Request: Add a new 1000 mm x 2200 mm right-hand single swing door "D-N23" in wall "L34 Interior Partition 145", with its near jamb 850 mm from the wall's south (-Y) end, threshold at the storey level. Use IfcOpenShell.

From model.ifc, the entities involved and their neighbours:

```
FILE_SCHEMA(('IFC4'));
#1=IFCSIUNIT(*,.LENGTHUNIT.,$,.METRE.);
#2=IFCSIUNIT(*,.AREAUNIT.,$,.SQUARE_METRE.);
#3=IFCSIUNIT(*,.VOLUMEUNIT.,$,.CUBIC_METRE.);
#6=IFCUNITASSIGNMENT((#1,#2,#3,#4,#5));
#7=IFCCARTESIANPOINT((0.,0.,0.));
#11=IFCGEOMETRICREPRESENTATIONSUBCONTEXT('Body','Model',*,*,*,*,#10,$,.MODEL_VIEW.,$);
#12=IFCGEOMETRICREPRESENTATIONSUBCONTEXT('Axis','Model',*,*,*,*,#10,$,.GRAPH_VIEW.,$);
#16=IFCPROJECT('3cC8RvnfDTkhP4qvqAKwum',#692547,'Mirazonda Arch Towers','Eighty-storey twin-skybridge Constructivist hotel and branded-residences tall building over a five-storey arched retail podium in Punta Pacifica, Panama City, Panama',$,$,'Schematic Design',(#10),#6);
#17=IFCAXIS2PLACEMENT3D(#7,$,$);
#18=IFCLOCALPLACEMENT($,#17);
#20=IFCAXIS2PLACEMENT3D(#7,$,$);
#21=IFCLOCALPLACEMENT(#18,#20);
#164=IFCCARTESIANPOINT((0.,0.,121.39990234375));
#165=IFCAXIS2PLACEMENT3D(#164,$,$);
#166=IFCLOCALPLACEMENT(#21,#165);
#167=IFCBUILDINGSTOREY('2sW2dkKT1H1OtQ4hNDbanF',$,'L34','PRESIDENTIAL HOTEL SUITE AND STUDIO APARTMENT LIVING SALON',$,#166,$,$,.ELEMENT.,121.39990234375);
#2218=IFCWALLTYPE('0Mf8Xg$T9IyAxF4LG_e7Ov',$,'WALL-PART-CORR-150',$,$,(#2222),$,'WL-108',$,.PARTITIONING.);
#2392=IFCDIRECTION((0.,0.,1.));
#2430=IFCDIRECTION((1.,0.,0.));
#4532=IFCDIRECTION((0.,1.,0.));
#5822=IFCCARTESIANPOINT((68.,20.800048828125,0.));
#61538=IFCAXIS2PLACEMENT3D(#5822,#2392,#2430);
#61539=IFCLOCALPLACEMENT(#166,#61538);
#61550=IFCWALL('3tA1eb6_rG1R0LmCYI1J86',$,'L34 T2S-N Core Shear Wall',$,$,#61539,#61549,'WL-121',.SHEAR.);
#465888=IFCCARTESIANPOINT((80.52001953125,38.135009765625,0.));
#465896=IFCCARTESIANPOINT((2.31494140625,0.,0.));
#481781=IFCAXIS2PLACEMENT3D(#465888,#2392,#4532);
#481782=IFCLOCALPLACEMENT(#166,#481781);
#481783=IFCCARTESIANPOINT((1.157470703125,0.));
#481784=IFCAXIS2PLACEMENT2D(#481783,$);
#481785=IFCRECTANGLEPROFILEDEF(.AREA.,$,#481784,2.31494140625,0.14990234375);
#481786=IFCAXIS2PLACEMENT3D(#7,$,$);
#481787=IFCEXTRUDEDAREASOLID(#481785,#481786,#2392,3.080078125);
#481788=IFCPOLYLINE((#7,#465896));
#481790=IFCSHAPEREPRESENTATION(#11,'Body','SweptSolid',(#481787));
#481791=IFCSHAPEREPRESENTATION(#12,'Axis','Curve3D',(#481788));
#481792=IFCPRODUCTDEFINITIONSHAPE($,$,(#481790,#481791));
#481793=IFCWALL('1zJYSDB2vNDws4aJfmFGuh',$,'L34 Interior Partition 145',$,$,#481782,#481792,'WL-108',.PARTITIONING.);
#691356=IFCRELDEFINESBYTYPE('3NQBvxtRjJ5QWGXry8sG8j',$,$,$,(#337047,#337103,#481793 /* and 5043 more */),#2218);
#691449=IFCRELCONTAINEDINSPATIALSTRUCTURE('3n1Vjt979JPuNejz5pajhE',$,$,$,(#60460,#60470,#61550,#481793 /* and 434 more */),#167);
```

```python
import numpy as np
import ifcopenshell
import ifcopenshell.api.feature
import ifcopenshell.api.geometry
import ifcopenshell.api.root
import ifcopenshell.api.spatial
import ifcopenshell.geom
import ifcopenshell.util.element
import ifcopenshell.util.placement
import ifcopenshell.util.representation
import ifcopenshell.util.shape
import ifcopenshell.util.unit

model = ifcopenshell.open("model.ifc")
unit_scale = ifcopenshell.util.unit.calculate_unit_scale(model)
settings = ifcopenshell.geom.settings()


def volume(element):
    """Net volume in cubic metres, openings subtracted."""
    shape = ifcopenshell.geom.create_shape(settings, element)
    return ifcopenshell.util.shape.get_volume(shape.geometry)


wall = model.by_guid("1zJYSDB2vNDws4aJfmFGuh")
storey = ifcopenshell.util.element.get_container(wall, ifc_class="IfcBuildingStorey")
context = ifcopenshell.util.representation.get_context(model, "Model", "Body", "MODEL_VIEW")
before = volume(wall)

width, height, from_end, sill = 1, 2.2, 0.85, 0.0  # metres

# The wall runs along its own X axis, and the end named is its -X end.
wall_shape = ifcopenshell.geom.create_shape(settings, wall)
x, y, z = ifcopenshell.util.shape.get_vertices(wall_shape.geometry).T
start = x.min() + from_end
face, thickness = float(y.min()), float(y.max() - y.min())
wall_matrix = ifcopenshell.util.placement.get_local_placement(wall.ObjectPlacement)
level = ifcopenshell.util.placement.get_local_placement(storey.ObjectPlacement)[2, 3]


def in_wall(x, y):
    """Placement at x, y metres in the wall's axes, at sill height."""
    matrix = wall_matrix.copy()
    matrix[:, 3] = wall_matrix @ np.array([x / unit_scale, y / unit_scale, 0.0, 1.0])
    matrix[2, 3] = level + sill / unit_scale
    return matrix


# Opening: a box that overshoots both wall faces by 50 mm.
opening = ifcopenshell.api.root.create_entity(model, ifc_class="IfcOpeningElement", predefined_type="OPENING")
box = ifcopenshell.api.geometry.add_wall_representation(
    model, context=context, length=width, height=height, thickness=thickness + 0.1
)
ifcopenshell.api.geometry.assign_representation(model, product=opening, representation=box)
ifcopenshell.api.geometry.edit_object_placement(model, product=opening, matrix=in_wall(start, face - 0.05), is_si=False)
ifcopenshell.api.feature.add_feature(model, feature=opening, element=wall)

door = ifcopenshell.api.root.create_entity(model, ifc_class="IfcDoor", name="D-N23", predefined_type="DOOR")
door.OverallWidth, door.OverallHeight = width / unit_scale, height / unit_scale
door.OperationType = "SINGLE_SWING_RIGHT"
body = ifcopenshell.api.geometry.add_door_representation(
    model,
    context=context,
    overall_width=door.OverallWidth,
    overall_height=door.OverallHeight,
    operation_type="SINGLE_SWING_RIGHT",
    lining_properties={"LiningDepth": thickness / unit_scale, "ThresholdDepth": thickness / unit_scale},
)
ifcopenshell.api.geometry.assign_representation(model, product=door, representation=body)
ifcopenshell.api.spatial.assign_container(model, products=[door], relating_structure=storey)
ifcopenshell.api.feature.add_filling(model, opening=opening, element=door)

# The lining spans the wall, so the door starts at the wall face.
ifcopenshell.api.geometry.edit_object_placement(model, product=door, matrix=in_wall(start, face), is_si=False)

after = volume(wall)

print(f"wall volume {before:.3f} -> {after:.3f} m3")

model.write("model-out.ifc")
```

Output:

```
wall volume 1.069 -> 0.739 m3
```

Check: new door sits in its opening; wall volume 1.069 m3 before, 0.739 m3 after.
